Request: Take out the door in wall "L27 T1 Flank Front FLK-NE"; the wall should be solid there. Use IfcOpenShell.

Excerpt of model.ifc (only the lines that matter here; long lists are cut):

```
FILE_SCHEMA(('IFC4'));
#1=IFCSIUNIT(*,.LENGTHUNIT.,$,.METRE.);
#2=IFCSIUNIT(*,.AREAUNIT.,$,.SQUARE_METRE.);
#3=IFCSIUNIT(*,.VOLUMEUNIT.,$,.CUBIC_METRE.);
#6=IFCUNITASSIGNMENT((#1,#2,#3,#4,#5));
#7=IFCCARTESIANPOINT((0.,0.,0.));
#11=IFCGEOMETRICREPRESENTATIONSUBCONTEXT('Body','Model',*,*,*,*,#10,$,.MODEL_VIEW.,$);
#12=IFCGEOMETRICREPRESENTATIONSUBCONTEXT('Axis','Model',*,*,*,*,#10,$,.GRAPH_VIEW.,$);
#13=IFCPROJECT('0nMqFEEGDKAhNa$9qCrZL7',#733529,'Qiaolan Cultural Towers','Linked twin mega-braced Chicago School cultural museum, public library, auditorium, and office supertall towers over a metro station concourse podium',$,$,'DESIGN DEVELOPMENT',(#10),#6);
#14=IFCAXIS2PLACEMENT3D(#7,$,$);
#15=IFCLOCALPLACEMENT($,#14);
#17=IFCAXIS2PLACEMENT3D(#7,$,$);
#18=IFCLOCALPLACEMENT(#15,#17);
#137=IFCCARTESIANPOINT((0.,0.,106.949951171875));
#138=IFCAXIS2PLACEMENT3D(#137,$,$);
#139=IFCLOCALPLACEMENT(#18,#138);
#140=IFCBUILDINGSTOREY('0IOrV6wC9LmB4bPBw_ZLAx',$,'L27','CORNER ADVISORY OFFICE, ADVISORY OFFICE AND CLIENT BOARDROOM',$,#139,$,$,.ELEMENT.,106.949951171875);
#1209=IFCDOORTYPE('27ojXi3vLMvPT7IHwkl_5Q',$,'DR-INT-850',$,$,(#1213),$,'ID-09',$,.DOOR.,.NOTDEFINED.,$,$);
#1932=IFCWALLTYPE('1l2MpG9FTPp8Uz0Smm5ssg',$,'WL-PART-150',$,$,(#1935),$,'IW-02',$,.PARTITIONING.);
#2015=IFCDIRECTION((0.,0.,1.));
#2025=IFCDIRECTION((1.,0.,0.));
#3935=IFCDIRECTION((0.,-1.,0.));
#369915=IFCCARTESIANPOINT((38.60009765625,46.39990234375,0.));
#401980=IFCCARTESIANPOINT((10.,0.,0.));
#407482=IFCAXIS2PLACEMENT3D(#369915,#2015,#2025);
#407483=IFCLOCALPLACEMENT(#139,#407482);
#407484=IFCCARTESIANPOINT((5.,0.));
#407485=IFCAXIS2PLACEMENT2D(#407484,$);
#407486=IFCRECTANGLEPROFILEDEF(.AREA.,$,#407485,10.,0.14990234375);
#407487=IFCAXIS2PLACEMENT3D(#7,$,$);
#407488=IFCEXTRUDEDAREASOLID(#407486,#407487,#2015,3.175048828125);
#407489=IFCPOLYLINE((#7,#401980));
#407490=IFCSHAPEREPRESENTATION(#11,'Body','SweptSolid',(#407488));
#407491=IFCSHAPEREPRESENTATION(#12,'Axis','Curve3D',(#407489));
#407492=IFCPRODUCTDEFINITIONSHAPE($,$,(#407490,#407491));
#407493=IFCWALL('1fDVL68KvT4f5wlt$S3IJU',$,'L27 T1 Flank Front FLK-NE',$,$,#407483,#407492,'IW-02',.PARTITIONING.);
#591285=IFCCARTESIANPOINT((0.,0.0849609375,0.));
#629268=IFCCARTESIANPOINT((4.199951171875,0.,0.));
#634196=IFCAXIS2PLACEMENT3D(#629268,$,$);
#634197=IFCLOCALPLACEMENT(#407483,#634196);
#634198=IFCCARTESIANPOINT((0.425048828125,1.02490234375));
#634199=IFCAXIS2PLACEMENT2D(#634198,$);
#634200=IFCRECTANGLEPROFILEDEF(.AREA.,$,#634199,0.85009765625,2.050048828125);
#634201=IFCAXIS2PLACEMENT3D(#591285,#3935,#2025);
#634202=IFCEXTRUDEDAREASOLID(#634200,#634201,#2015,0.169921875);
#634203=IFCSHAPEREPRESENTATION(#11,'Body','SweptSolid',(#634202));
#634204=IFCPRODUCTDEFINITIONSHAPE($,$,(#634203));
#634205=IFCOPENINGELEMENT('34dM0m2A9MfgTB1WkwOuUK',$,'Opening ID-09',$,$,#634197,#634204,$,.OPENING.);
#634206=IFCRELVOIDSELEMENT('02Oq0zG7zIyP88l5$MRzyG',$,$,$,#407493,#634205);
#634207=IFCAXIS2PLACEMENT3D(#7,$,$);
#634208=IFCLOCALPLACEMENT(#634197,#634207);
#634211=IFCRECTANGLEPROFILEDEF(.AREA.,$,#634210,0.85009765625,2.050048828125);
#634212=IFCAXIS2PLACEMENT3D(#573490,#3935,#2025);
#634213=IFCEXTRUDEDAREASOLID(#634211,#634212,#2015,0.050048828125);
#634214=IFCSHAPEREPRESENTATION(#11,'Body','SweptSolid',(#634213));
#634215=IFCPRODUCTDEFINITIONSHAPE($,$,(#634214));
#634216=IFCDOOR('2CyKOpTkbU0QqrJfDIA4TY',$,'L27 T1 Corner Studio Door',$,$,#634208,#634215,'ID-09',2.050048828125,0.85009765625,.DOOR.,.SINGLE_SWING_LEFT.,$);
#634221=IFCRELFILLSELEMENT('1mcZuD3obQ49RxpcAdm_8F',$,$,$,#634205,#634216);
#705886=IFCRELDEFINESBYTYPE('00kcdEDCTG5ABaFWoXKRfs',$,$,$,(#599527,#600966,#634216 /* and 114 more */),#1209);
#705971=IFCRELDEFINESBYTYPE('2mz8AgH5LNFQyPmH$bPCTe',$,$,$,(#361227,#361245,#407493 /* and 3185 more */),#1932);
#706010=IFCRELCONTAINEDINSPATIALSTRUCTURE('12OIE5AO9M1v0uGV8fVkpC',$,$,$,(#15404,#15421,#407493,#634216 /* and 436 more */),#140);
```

```python
import ifcopenshell
import ifcopenshell.api.feature
import ifcopenshell.api.root
import ifcopenshell.geom
import ifcopenshell.util.shape

model = ifcopenshell.open("model.ifc")
settings = ifcopenshell.geom.settings()


def volume(element):
    """Net volume in cubic metres, openings subtracted."""
    shape = ifcopenshell.geom.create_shape(settings, element)
    return ifcopenshell.util.shape.get_volume(shape.geometry)


door = model.by_id(634216)
opening = door.FillsVoids[0].RelatingOpeningElement
wall = opening.VoidsElements[0].RelatingBuildingElement
before = volume(wall)

ifcopenshell.api.root.remove_product(model, product=door)
ifcopenshell.api.feature.remove_feature(model, feature=opening)

after = volume(wall)

print(f"wall volume {before:.3f} -> {after:.3f} m3")

model.write("model_rev.ifc")
```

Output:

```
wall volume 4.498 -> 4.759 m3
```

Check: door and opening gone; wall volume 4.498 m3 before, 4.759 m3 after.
